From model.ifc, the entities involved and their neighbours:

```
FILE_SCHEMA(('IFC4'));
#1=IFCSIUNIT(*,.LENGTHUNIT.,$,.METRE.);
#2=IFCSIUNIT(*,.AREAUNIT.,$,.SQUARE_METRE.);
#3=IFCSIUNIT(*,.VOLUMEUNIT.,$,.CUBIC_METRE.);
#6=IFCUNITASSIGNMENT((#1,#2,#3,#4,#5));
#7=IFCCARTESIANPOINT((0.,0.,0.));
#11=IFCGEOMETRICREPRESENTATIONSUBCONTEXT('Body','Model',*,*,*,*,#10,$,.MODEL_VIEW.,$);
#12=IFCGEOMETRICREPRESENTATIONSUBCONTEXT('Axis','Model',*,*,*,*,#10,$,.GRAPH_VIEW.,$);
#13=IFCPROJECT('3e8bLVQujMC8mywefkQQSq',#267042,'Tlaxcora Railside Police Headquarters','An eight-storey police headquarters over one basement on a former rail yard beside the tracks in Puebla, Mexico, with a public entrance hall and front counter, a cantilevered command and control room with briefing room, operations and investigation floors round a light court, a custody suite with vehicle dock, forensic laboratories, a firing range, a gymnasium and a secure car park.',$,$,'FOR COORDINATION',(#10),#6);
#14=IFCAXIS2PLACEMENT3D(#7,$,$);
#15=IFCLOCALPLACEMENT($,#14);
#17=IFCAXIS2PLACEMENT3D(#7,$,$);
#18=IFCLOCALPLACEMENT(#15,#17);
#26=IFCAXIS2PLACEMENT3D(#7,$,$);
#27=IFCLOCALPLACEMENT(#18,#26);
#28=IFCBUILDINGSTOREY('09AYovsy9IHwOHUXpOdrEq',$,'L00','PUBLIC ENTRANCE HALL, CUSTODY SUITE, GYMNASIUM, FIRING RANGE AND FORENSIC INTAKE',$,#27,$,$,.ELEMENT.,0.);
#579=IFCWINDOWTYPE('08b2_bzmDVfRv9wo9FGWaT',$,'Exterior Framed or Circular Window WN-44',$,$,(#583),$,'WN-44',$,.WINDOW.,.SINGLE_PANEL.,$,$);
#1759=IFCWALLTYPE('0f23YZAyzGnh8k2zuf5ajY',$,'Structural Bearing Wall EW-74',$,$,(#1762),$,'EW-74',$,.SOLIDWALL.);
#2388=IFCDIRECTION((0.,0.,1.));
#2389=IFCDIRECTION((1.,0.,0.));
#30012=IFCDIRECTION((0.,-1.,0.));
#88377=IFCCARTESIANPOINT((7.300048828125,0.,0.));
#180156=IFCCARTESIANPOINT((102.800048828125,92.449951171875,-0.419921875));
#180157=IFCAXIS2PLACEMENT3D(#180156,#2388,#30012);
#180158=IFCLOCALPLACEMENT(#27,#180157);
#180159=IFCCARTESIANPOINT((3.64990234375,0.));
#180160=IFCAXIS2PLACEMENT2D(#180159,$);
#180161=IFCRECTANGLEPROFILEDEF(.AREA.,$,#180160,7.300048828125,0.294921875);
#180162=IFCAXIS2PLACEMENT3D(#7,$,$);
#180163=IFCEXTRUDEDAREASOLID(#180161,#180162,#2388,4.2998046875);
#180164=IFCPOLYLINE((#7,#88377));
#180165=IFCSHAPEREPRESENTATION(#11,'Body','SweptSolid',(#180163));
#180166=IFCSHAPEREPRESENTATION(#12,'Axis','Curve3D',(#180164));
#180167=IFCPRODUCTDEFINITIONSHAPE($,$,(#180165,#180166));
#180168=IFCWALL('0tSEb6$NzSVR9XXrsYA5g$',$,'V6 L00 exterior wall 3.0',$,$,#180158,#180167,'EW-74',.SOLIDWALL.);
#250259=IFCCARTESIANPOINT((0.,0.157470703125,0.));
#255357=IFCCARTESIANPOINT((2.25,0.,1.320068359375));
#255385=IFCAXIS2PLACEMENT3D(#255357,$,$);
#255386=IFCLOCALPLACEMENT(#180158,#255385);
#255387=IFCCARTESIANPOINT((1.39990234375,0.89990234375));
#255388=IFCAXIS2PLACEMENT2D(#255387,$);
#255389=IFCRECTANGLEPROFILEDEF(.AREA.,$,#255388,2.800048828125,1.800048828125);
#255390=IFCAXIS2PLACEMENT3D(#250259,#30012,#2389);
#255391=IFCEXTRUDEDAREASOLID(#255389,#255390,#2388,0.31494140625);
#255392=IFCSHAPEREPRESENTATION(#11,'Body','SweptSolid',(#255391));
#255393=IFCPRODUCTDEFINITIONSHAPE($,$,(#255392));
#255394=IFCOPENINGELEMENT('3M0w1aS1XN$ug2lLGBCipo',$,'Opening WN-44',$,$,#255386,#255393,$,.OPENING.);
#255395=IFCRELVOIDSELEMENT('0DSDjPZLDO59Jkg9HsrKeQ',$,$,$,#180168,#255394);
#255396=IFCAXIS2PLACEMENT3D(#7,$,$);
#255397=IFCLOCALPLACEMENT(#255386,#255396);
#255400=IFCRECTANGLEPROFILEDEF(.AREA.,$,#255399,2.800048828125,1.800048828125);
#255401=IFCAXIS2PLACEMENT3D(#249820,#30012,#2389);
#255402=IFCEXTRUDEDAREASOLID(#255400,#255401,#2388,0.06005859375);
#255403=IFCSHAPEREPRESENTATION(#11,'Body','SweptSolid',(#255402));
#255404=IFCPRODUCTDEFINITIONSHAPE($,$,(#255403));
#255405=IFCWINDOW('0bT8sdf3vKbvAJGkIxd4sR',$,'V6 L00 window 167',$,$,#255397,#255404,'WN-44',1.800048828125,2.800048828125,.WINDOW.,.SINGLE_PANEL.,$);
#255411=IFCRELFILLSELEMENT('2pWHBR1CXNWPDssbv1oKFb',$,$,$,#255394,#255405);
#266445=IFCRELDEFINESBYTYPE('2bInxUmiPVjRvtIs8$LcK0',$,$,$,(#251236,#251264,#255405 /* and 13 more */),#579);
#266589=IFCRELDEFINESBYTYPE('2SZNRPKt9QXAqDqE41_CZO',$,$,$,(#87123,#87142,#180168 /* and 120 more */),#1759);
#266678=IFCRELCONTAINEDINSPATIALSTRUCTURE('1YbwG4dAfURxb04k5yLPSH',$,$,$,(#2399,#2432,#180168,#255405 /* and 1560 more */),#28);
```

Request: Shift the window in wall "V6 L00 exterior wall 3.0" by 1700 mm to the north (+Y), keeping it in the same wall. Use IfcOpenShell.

```python
import ifcopenshell
import ifcopenshell.api.geometry
import ifcopenshell.util.placement

model = ifcopenshell.open("model.ifc")

window = model.by_id(255405)
opening = window.FillsVoids[0].RelatingOpeningElement
wall = opening.VoidsElements[0].RelatingBuildingElement

wall_matrix = ifcopenshell.util.placement.get_local_placement(wall.ObjectPlacement)
shift = wall_matrix[:3, 0] * -1.7
before = ifcopenshell.util.placement.get_local_placement(window.ObjectPlacement)[:3, 3].copy()

# The window is placed relative to its opening, so it follows when the opening moves.
matrix = ifcopenshell.util.placement.get_local_placement(opening.ObjectPlacement)
matrix[:3, 3] += shift
ifcopenshell.api.geometry.edit_object_placement(
    model, product=opening, matrix=matrix, is_si=False, should_transform_children=True
)

after = ifcopenshell.util.placement.get_local_placement(window.ObjectPlacement)[:3, 3]
print("window moved by", (after - before).round(3) + 0.0)

model.write("model_rev.ifc")
```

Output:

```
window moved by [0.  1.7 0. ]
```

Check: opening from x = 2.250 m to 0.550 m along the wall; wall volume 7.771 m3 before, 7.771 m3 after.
